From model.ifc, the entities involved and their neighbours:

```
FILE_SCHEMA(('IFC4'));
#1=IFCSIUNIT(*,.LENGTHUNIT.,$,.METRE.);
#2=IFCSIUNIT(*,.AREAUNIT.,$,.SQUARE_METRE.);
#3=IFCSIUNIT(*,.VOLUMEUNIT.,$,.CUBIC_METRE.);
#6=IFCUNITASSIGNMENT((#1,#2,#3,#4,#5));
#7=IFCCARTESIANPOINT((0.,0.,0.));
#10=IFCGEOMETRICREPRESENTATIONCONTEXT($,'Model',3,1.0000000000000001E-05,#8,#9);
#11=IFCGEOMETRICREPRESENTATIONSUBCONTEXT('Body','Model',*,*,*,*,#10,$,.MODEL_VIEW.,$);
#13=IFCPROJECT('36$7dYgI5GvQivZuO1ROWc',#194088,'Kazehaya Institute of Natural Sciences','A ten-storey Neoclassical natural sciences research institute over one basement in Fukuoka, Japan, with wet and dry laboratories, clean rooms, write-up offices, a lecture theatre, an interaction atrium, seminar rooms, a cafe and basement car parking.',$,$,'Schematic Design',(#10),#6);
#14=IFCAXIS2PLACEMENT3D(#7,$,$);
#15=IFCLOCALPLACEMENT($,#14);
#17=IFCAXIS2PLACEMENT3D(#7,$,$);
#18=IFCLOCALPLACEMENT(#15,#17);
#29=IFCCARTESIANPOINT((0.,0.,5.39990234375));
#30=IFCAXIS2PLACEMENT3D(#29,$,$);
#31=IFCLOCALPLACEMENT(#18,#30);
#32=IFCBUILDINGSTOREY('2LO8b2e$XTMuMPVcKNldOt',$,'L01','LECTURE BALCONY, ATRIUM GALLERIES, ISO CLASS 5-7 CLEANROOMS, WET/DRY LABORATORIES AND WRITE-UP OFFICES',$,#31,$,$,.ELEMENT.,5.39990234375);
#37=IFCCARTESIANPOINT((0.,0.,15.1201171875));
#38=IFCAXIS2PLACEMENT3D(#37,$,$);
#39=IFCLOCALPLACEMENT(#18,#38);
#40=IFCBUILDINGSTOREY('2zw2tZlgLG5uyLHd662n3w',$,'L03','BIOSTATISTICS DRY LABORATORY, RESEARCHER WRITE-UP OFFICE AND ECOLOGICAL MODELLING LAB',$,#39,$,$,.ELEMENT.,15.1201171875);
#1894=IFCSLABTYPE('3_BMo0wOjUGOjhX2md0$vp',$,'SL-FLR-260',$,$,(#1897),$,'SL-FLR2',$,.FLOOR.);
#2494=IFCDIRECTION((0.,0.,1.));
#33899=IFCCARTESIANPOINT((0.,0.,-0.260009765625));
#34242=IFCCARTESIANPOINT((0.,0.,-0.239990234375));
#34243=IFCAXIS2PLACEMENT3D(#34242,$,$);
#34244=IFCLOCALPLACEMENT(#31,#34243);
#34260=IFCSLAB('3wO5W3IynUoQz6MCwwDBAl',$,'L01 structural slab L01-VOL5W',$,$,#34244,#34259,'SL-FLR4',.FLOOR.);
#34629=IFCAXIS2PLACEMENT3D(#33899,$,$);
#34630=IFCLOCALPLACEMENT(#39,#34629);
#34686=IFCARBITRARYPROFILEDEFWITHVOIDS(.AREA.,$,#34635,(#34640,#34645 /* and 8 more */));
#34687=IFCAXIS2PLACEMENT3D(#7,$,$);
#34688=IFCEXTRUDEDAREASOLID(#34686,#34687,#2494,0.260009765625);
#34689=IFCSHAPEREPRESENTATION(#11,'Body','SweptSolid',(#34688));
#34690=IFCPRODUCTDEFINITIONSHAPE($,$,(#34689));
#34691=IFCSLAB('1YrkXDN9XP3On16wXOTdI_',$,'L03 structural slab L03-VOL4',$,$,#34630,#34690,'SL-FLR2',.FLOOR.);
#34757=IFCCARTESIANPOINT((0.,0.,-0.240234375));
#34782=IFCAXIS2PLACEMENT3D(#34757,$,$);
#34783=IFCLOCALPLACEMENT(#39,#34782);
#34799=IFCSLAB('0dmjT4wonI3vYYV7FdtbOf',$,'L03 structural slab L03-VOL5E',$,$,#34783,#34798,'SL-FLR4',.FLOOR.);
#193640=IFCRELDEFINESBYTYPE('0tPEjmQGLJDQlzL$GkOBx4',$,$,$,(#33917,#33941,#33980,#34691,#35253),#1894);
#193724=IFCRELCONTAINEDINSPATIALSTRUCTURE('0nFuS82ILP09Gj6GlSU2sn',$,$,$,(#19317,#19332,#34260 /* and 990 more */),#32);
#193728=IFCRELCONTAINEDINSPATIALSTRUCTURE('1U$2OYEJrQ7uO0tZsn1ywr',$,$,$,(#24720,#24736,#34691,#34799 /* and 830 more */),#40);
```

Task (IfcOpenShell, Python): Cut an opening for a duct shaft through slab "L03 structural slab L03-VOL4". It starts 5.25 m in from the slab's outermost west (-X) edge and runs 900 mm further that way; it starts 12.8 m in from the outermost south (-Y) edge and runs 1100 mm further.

```python
import numpy as np
import ifcopenshell
import ifcopenshell.api.feature
import ifcopenshell.api.geometry
import ifcopenshell.api.root
import ifcopenshell.geom
import ifcopenshell.util.placement
import ifcopenshell.util.representation
import ifcopenshell.util.shape
import ifcopenshell.util.unit

model = ifcopenshell.open("model.ifc")
unit_scale = ifcopenshell.util.unit.calculate_unit_scale(model)
settings = ifcopenshell.geom.settings()


def volume(element):
    """Net volume in cubic metres, openings subtracted."""
    shape = ifcopenshell.geom.create_shape(settings, element)
    return ifcopenshell.util.shape.get_volume(shape.geometry)


slab = model.by_id(34691)
before = volume(slab)

# Extent in the slab's own axes, in metres. The edges named are its -X and -Y sides.
slab_shape = ifcopenshell.geom.create_shape(settings, slab)
vertices = ifcopenshell.util.shape.get_vertices(slab_shape.geometry)
x_min, y_min, bottom = vertices.min(axis=0)
top = vertices[:, 2].max()

opening = ifcopenshell.api.root.create_entity(model, ifc_class="IfcOpeningElement", name="Duct shaft opening", predefined_type="OPENING")
context = ifcopenshell.util.representation.get_context(model, "Model", "Body", "MODEL_VIEW")
width, depth = 0.9, 1.1
outline = [(0.0, 0.0), (width, 0.0), (width, depth), (0.0, depth), (0.0, 0.0)]
# Overshoot both faces by 50 mm so the cut is clean.
shape = ifcopenshell.api.geometry.add_slab_representation(
    model, context=context, depth=top - bottom + 0.1, polyline=outline
)
ifcopenshell.api.geometry.assign_representation(model, product=opening, representation=shape)

matrix = ifcopenshell.util.placement.get_local_placement(slab.ObjectPlacement)
matrix[:, 3] = matrix @ np.append(np.array([x_min + 5.25, y_min + 12.8, bottom - 0.05]) / unit_scale, 1.0)
ifcopenshell.api.geometry.edit_object_placement(model, product=opening, matrix=matrix, is_si=False)
ifcopenshell.api.feature.add_feature(model, feature=opening, element=slab)

after = volume(slab)

print(f"slab volume {before:.3f} -> {after:.3f} m3")

model.write("model_updated.ifc")
```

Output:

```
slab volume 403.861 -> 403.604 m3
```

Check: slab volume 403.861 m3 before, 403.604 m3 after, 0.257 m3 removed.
